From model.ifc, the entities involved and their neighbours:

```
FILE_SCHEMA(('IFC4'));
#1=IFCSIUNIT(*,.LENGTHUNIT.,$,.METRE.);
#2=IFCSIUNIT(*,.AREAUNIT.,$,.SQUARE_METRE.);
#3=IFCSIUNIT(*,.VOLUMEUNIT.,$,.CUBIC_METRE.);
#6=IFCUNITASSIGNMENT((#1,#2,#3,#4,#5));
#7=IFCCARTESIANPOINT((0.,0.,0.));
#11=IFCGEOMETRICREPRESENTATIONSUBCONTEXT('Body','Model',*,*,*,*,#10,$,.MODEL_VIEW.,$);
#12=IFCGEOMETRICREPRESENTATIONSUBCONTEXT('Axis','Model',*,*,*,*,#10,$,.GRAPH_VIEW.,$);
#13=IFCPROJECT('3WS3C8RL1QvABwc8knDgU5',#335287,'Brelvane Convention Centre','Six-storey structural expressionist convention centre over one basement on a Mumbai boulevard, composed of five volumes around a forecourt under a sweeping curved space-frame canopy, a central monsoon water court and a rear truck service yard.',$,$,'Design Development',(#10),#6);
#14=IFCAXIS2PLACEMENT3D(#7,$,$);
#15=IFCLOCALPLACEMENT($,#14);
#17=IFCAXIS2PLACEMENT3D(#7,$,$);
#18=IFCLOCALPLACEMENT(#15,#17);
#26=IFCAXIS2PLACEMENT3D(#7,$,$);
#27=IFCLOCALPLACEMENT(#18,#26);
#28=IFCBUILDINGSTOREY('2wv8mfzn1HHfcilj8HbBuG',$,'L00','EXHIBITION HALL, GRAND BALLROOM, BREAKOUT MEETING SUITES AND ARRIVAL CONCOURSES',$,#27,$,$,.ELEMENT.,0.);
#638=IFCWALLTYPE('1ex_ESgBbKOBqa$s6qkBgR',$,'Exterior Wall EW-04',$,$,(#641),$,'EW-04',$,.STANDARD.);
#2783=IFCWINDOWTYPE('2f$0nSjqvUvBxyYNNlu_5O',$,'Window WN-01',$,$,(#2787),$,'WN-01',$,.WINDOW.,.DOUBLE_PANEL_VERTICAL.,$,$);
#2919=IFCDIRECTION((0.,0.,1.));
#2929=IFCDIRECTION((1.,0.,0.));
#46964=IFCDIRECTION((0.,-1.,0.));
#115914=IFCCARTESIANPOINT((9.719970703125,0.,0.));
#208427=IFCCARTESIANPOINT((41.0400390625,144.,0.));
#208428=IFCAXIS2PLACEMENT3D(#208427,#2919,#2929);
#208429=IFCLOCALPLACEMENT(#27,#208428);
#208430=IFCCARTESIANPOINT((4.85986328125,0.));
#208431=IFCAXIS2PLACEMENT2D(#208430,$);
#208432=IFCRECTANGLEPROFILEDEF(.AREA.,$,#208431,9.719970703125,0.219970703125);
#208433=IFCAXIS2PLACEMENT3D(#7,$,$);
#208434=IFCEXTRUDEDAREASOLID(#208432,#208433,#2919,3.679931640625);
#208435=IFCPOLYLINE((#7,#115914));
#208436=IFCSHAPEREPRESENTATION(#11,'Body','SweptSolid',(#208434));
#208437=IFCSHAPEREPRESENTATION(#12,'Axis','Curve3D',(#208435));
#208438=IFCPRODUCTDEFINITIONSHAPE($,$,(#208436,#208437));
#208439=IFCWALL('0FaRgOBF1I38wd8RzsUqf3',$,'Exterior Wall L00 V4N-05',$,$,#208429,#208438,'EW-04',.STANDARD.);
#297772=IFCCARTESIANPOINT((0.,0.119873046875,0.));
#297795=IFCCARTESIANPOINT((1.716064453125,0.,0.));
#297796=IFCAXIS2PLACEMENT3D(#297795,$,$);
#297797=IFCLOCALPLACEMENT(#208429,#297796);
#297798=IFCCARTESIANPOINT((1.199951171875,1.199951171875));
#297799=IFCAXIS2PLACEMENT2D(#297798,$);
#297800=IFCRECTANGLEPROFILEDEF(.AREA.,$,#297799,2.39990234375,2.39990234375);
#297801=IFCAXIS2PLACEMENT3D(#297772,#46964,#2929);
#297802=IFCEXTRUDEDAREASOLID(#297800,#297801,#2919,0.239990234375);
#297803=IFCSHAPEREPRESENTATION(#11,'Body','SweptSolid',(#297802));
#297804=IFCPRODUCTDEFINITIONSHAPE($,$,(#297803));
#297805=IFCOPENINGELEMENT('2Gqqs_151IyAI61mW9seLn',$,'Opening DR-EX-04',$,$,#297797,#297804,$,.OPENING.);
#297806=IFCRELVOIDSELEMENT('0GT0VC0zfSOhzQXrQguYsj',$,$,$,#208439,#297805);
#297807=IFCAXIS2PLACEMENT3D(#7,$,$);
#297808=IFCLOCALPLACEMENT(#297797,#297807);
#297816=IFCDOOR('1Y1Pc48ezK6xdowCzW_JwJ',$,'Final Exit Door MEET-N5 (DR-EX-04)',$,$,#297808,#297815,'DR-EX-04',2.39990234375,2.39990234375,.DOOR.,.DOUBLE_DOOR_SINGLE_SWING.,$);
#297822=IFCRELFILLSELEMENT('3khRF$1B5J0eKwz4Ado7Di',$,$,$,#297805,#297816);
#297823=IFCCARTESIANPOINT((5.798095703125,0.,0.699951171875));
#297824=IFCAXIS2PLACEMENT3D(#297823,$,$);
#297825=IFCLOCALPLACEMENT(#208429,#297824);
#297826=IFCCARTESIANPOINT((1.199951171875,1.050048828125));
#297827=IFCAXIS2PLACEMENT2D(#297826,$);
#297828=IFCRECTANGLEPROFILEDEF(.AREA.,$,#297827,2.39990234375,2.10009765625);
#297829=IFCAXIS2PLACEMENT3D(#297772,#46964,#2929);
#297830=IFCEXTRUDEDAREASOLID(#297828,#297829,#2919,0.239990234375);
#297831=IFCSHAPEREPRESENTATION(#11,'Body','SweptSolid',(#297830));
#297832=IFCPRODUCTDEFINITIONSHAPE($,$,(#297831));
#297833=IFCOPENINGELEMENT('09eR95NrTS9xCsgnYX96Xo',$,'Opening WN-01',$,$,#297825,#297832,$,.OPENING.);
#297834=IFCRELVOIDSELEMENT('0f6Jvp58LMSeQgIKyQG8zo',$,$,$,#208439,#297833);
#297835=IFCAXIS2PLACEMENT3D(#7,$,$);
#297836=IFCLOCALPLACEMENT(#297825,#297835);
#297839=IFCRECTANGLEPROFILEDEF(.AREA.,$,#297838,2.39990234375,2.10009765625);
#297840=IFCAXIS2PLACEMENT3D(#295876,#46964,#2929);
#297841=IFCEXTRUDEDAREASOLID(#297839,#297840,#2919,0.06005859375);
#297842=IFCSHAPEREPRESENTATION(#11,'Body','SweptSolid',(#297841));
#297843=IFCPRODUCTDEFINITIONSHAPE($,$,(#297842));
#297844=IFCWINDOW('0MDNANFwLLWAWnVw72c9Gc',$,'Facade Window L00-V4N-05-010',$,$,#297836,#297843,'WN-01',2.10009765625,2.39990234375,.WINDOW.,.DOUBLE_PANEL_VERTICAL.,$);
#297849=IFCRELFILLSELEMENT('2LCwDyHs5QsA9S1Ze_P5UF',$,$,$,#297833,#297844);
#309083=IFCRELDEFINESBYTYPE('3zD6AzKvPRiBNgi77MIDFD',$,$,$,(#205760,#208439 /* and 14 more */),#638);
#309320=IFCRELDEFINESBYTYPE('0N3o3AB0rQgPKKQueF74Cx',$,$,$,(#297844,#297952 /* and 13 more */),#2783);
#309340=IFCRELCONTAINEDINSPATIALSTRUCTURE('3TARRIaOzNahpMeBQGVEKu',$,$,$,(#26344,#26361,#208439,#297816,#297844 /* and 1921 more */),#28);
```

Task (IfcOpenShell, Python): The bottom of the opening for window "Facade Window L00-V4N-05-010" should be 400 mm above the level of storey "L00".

```python
import numpy as np
import ifcopenshell
import ifcopenshell.api.geometry
import ifcopenshell.geom
import ifcopenshell.util.element
import ifcopenshell.util.placement
import ifcopenshell.util.shape
import ifcopenshell.util.unit

model = ifcopenshell.open("model.ifc")
unit_scale = ifcopenshell.util.unit.calculate_unit_scale(model)

window = model.by_id(297844)
opening = window.FillsVoids[0].RelatingOpeningElement
storey = ifcopenshell.util.element.get_container(window, ifc_class="IfcBuildingStorey")
level = ifcopenshell.util.placement.get_local_placement(storey.ObjectPlacement)[2, 3]

# The opening's origin need not be at the sill, so measure its lowest point.
shape = ifcopenshell.geom.create_shape(ifcopenshell.geom.settings(), opening)
bottom = ifcopenshell.util.shape.get_shape_bottom_elevation(shape, shape.geometry) / unit_scale
dz = level + 0.4 / unit_scale - bottom

shift = np.array([0.0, 0.0, dz])
# The window is placed relative to its opening, so it follows when the opening moves.
matrix = ifcopenshell.util.placement.get_local_placement(opening.ObjectPlacement)
matrix[:3, 3] += shift
ifcopenshell.api.geometry.edit_object_placement(
    model, product=opening, matrix=matrix, is_si=False, should_transform_children=True
)

print(f"moved by {dz * unit_scale:+.3f} m")

model.write("model_rev.ifc")
```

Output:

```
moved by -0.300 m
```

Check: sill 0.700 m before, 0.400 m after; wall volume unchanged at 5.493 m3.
